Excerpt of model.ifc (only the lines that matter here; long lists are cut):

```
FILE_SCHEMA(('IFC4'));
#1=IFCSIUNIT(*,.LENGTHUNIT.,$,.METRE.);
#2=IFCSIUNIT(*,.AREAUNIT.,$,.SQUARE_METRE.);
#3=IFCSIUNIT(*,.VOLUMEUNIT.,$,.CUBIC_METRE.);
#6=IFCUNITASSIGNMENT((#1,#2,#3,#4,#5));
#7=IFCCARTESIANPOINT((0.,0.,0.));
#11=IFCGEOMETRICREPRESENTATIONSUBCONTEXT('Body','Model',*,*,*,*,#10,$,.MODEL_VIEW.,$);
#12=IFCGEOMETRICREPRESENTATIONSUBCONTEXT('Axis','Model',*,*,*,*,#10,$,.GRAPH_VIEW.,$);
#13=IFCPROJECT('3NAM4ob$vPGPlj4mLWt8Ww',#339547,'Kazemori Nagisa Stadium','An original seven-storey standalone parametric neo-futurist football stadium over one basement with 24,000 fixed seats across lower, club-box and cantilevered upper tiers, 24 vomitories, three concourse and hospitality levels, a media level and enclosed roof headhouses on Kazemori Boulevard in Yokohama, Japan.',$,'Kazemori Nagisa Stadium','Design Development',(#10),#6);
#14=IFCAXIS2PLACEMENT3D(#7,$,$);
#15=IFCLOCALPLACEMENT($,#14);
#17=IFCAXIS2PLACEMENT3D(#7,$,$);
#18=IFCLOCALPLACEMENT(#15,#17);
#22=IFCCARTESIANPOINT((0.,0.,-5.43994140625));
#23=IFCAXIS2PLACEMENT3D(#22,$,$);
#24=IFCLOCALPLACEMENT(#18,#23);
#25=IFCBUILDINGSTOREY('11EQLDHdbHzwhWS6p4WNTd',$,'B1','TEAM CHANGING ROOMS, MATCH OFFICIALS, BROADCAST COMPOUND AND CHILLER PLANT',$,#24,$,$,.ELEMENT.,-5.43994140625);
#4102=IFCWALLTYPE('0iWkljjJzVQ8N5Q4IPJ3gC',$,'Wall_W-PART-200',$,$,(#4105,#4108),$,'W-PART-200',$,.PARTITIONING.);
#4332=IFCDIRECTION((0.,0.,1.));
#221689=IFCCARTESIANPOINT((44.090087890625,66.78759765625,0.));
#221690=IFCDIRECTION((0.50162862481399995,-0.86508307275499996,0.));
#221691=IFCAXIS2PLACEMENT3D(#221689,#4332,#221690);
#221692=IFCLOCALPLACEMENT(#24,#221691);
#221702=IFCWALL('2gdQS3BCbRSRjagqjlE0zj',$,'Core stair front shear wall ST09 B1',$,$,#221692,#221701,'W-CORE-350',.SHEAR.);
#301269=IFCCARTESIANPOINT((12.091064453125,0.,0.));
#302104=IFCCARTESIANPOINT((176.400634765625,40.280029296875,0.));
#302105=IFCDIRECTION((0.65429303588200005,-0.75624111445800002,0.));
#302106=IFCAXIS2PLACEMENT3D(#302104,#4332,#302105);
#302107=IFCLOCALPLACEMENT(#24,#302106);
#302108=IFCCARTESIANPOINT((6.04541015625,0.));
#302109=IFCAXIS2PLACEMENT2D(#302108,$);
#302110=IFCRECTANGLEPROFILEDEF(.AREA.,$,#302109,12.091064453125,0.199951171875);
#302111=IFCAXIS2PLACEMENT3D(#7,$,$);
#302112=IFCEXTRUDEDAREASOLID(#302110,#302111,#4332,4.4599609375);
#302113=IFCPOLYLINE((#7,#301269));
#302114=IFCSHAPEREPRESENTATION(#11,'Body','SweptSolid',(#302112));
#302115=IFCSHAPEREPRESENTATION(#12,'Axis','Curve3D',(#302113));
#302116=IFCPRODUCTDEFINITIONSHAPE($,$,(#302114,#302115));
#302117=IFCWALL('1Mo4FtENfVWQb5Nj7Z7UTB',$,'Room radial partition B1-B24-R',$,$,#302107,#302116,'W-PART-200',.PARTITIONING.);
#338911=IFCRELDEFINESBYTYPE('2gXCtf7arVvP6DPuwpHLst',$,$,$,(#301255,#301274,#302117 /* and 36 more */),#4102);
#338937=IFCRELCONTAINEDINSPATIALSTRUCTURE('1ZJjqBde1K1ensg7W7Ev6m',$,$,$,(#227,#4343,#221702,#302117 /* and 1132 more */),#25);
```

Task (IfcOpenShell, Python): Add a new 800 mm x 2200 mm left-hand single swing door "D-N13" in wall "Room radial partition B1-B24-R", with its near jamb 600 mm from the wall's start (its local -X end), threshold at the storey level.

```python
import numpy as np
import ifcopenshell
import ifcopenshell.api.feature
import ifcopenshell.api.geometry
import ifcopenshell.api.root
import ifcopenshell.api.spatial
import ifcopenshell.geom
import ifcopenshell.util.element
import ifcopenshell.util.placement
import ifcopenshell.util.representation
import ifcopenshell.util.shape
import ifcopenshell.util.unit

model = ifcopenshell.open("model.ifc")
unit_scale = ifcopenshell.util.unit.calculate_unit_scale(model)
settings = ifcopenshell.geom.settings()


def volume(element):
    """Net volume in cubic metres, openings subtracted."""
    shape = ifcopenshell.geom.create_shape(settings, element)
    return ifcopenshell.util.shape.get_volume(shape.geometry)


wall = model.by_guid("1Mo4FtENfVWQb5Nj7Z7UTB")
storey = ifcopenshell.util.element.get_container(wall, ifc_class="IfcBuildingStorey")
context = ifcopenshell.util.representation.get_context(model, "Model", "Body", "MODEL_VIEW")
before = volume(wall)

width, height, from_end, sill = 0.8, 2.2, 0.6, 0.0  # metres

# The wall runs along its own X axis, and the end named is its -X end.
wall_shape = ifcopenshell.geom.create_shape(settings, wall)
x, y, z = ifcopenshell.util.shape.get_vertices(wall_shape.geometry).T
start = x.min() + from_end
face, thickness = float(y.min()), float(y.max() - y.min())
wall_matrix = ifcopenshell.util.placement.get_local_placement(wall.ObjectPlacement)
level = ifcopenshell.util.placement.get_local_placement(storey.ObjectPlacement)[2, 3]


def in_wall(x, y):
    """Placement at x, y metres in the wall's axes, at sill height."""
    matrix = wall_matrix.copy()
    matrix[:, 3] = wall_matrix @ np.array([x / unit_scale, y / unit_scale, 0.0, 1.0])
    matrix[2, 3] = level + sill / unit_scale
    return matrix


# Opening: a box that overshoots both wall faces by 50 mm.
opening = ifcopenshell.api.root.create_entity(model, ifc_class="IfcOpeningElement", predefined_type="OPENING")
box = ifcopenshell.api.geometry.add_wall_representation(
    model, context=context, length=width, height=height, thickness=thickness + 0.1
)
ifcopenshell.api.geometry.assign_representation(model, product=opening, representation=box)
ifcopenshell.api.geometry.edit_object_placement(model, product=opening, matrix=in_wall(start, face - 0.05), is_si=False)
ifcopenshell.api.feature.add_feature(model, feature=opening, element=wall)

door = ifcopenshell.api.root.create_entity(model, ifc_class="IfcDoor", name="D-N13", predefined_type="DOOR")
door.OverallWidth, door.OverallHeight = width / unit_scale, height / unit_scale
door.OperationType = "SINGLE_SWING_LEFT"
body = ifcopenshell.api.geometry.add_door_representation(
    model,
    context=context,
    overall_width=door.OverallWidth,
    overall_height=door.OverallHeight,
    operation_type="SINGLE_SWING_LEFT",
    lining_properties={"LiningDepth": thickness / unit_scale, "ThresholdDepth": thickness / unit_scale},
)
ifcopenshell.api.geometry.assign_representation(model, product=door, representation=body)
ifcopenshell.api.spatial.assign_container(model, products=[door], relating_structure=storey)
ifcopenshell.api.feature.add_filling(model, opening=opening, element=door)

# The lining spans the wall, so the door starts at the wall face.
ifcopenshell.api.geometry.edit_object_placement(model, product=door, matrix=in_wall(start, face), is_si=False)

after = volume(wall)

print(f"wall volume {before:.3f} -> {after:.3f} m3")

model.write("model_updated.ifc")
```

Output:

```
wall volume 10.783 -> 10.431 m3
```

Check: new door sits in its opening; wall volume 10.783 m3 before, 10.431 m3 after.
